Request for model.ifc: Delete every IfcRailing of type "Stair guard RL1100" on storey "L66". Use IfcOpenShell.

First a look at what the model holds.

```python
import ifcopenshell
import ifcopenshell.util.element

model = ifcopenshell.open("model.ifc")
print(model.schema)
storey = next(s for s in model.by_type("IfcBuildingStorey") if s.Name == "L66")
railings = [e for e in ifcopenshell.util.element.get_decomposition(storey) if e.is_a("IfcRailing")]
seen = {}
for e in railings:
    element_type = ifcopenshell.util.element.get_type(e)
    name = element_type.Name if element_type not in (None, e) else None
    seen[name] = seen.get(name, 0) + 1
for name, count in sorted(seen.items(), key=str):
    print(count, "x", name)
```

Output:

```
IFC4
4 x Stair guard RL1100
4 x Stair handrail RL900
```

```python
import ifcopenshell
import ifcopenshell.api.root
import ifcopenshell.util.element

model = ifcopenshell.open("model.ifc")

storey = next(s for s in model.by_type("IfcBuildingStorey") if s.Name == "L66")
railings = [e for e in ifcopenshell.util.element.get_decomposition(storey) if e.is_a("IfcRailing")]
targets = [e for e in railings if (t := ifcopenshell.util.element.get_type(e)) not in (None, e) and t.Name == "Stair guard RL1100"]

for e in targets:
    ifcopenshell.api.root.remove_product(model, product=e)
print(len(targets), "removed")

model.write("model_rev.ifc")
```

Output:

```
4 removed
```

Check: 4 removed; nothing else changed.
